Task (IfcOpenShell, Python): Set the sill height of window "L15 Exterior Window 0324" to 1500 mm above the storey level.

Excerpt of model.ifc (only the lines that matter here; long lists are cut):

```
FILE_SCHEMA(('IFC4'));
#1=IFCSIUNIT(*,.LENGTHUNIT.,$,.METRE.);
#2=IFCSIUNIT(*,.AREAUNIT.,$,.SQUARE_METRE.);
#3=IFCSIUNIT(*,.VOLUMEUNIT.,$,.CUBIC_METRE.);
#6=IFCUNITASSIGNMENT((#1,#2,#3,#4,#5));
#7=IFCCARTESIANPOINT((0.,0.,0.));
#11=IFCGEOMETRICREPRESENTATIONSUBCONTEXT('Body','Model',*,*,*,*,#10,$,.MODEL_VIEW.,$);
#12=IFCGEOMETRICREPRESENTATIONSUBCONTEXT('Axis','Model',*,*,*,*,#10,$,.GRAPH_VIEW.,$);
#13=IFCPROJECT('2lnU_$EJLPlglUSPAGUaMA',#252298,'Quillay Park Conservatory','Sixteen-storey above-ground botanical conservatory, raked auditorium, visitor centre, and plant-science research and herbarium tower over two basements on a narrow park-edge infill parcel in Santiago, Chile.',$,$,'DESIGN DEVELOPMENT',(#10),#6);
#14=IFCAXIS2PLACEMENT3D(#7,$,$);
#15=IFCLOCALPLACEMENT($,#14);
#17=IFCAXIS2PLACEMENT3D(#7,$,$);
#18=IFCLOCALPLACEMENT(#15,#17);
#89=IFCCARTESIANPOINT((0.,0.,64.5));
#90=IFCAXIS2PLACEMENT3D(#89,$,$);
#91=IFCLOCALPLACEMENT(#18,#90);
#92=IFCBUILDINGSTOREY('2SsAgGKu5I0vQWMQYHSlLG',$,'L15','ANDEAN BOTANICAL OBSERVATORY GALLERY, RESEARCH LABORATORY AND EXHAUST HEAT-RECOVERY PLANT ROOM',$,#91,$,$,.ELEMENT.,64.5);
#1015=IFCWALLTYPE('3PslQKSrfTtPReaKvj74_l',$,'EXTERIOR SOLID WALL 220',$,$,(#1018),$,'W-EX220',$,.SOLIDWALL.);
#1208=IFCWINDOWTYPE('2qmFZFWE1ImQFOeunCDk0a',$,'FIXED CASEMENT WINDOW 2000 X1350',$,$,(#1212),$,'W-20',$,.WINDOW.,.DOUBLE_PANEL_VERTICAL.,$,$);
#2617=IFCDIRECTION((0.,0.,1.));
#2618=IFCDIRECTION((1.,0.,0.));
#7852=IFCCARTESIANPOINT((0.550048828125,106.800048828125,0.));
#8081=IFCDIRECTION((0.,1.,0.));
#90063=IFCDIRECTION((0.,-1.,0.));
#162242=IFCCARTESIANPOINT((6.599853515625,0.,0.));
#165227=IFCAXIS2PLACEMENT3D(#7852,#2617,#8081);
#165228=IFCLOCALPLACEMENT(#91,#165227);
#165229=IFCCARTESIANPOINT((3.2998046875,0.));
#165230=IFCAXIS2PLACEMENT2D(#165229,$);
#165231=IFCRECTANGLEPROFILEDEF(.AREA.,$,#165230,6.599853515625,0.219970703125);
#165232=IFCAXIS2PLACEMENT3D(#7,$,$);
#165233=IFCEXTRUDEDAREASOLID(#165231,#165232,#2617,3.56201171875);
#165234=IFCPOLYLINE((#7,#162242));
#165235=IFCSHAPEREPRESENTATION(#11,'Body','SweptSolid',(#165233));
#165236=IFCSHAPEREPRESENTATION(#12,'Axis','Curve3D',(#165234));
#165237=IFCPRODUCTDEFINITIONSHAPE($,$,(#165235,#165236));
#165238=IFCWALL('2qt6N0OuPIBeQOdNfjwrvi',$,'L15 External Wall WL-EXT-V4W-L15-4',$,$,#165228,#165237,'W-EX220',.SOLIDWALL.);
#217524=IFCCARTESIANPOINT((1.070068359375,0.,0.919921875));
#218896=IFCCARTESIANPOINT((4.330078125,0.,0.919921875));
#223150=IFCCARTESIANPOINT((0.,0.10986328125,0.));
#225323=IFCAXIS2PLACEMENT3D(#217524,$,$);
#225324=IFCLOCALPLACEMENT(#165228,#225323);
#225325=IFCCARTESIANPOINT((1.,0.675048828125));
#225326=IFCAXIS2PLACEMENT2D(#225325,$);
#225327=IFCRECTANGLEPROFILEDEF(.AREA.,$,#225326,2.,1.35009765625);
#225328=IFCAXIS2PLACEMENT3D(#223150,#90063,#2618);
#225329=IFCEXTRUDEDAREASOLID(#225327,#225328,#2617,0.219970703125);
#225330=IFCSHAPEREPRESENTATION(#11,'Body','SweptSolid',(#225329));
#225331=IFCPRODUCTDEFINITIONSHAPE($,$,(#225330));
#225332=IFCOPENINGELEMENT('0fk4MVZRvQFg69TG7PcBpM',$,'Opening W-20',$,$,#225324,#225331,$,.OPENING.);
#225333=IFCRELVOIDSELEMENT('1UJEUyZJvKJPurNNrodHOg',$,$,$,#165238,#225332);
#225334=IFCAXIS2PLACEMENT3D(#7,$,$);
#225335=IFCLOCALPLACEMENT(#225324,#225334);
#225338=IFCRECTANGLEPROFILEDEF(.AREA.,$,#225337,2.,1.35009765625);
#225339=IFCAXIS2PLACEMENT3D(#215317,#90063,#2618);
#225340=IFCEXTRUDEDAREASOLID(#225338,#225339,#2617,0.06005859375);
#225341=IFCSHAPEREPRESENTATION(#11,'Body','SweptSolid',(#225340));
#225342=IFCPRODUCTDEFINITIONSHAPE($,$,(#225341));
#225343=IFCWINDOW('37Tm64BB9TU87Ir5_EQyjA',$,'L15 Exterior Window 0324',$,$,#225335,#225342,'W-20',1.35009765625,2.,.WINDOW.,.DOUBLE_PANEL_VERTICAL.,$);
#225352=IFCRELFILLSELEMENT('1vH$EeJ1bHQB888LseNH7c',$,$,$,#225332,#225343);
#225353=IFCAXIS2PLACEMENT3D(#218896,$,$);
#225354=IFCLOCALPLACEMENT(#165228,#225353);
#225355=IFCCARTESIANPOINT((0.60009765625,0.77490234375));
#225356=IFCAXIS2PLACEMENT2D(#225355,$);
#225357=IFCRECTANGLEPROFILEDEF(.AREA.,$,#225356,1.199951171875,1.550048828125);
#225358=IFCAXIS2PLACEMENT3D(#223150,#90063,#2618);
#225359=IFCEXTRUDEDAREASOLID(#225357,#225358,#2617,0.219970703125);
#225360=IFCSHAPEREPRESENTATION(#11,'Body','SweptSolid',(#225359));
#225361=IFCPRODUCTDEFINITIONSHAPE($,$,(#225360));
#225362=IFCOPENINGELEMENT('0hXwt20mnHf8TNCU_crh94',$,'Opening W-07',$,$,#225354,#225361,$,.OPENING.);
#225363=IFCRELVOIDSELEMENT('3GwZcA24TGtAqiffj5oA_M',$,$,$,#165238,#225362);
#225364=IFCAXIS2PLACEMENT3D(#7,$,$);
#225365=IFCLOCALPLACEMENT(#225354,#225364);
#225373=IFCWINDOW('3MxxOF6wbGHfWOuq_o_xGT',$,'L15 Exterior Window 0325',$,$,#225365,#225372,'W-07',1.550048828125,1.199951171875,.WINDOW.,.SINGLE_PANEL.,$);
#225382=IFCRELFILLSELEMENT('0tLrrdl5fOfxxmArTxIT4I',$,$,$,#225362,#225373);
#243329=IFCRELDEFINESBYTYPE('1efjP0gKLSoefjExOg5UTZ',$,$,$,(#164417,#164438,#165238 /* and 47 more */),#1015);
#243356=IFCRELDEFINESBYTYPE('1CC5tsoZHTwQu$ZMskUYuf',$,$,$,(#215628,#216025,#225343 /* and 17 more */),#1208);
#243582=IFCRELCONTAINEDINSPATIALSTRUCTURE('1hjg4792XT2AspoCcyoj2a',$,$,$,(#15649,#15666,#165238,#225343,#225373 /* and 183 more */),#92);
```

```python
import numpy as np
import ifcopenshell
import ifcopenshell.api.geometry
import ifcopenshell.geom
import ifcopenshell.util.element
import ifcopenshell.util.placement
import ifcopenshell.util.shape
import ifcopenshell.util.unit

model = ifcopenshell.open("model.ifc")
unit_scale = ifcopenshell.util.unit.calculate_unit_scale(model)

window = model.by_guid("37Tm64BB9TU87Ir5_EQyjA")
opening = window.FillsVoids[0].RelatingOpeningElement
storey = ifcopenshell.util.element.get_container(window, ifc_class="IfcBuildingStorey")
level = ifcopenshell.util.placement.get_local_placement(storey.ObjectPlacement)[2, 3]

# The opening's origin need not be at the sill, so measure its lowest point.
shape = ifcopenshell.geom.create_shape(ifcopenshell.geom.settings(), opening)
bottom = ifcopenshell.util.shape.get_shape_bottom_elevation(shape, shape.geometry) / unit_scale
dz = level + 1.5 - bottom

shift = np.array([0.0, 0.0, dz])
# The window is placed relative to its opening, so it follows when the opening moves.
matrix = ifcopenshell.util.placement.get_local_placement(opening.ObjectPlacement)
matrix[:3, 3] += shift
ifcopenshell.api.geometry.edit_object_placement(
    model, product=opening, matrix=matrix, is_si=False, should_transform_children=True
)

print(f"moved by {dz * unit_scale:+.3f} m")

model.write("model_edited.ifc")
```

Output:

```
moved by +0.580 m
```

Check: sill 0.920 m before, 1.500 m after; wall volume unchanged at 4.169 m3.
